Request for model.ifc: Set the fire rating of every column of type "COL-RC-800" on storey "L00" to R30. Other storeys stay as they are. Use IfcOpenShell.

First a look at what the model holds.

```python
import ifcopenshell
import ifcopenshell.util.element

model = ifcopenshell.open("model.ifc")
print(model.schema)
storey = next(s for s in model.by_type("IfcBuildingStorey") if s.Name == "L00")
columns = [e for e in ifcopenshell.util.element.get_decomposition(storey) if e.is_a("IfcColumn")]
seen = {}
for e in columns:
    element_type = ifcopenshell.util.element.get_type(e)
    key = (element_type.Name if element_type != e and element_type else None, ifcopenshell.util.element.get_pset(e, "Pset_ColumnCommon", "FireRating"))
    seen[key] = seen.get(key, 0) + 1
for (name, value), count in sorted(seen.items(), key=str):
    print(count, "x", name, "|", value)
```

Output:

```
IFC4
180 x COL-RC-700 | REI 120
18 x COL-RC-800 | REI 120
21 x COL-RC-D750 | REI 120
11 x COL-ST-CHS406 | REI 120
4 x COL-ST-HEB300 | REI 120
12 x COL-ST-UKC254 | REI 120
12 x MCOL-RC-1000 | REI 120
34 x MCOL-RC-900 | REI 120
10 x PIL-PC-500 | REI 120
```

```python
import ifcopenshell
import ifcopenshell.api.pset
import ifcopenshell.util.element

model = ifcopenshell.open("model.ifc")

storey = next(s for s in model.by_type("IfcBuildingStorey") if s.Name == "L00")
columns = [e for e in ifcopenshell.util.element.get_decomposition(storey) if e.is_a("IfcColumn")]

count = 0
for e in columns:
    element_type = ifcopenshell.util.element.get_type(e)
    if element_type in (None, e) or element_type.Name != "COL-RC-800":
        continue
    # add_pset returns the element's existing set when there is one.
    pset = ifcopenshell.api.pset.add_pset(model, product=e, name="Pset_ColumnCommon")
    ifcopenshell.api.pset.edit_pset(model, pset=pset, properties={"FireRating": "R30"})
    count += 1

print(count, "columns updated")

model.write("model-out.ifc")
```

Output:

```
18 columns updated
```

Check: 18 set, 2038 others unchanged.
